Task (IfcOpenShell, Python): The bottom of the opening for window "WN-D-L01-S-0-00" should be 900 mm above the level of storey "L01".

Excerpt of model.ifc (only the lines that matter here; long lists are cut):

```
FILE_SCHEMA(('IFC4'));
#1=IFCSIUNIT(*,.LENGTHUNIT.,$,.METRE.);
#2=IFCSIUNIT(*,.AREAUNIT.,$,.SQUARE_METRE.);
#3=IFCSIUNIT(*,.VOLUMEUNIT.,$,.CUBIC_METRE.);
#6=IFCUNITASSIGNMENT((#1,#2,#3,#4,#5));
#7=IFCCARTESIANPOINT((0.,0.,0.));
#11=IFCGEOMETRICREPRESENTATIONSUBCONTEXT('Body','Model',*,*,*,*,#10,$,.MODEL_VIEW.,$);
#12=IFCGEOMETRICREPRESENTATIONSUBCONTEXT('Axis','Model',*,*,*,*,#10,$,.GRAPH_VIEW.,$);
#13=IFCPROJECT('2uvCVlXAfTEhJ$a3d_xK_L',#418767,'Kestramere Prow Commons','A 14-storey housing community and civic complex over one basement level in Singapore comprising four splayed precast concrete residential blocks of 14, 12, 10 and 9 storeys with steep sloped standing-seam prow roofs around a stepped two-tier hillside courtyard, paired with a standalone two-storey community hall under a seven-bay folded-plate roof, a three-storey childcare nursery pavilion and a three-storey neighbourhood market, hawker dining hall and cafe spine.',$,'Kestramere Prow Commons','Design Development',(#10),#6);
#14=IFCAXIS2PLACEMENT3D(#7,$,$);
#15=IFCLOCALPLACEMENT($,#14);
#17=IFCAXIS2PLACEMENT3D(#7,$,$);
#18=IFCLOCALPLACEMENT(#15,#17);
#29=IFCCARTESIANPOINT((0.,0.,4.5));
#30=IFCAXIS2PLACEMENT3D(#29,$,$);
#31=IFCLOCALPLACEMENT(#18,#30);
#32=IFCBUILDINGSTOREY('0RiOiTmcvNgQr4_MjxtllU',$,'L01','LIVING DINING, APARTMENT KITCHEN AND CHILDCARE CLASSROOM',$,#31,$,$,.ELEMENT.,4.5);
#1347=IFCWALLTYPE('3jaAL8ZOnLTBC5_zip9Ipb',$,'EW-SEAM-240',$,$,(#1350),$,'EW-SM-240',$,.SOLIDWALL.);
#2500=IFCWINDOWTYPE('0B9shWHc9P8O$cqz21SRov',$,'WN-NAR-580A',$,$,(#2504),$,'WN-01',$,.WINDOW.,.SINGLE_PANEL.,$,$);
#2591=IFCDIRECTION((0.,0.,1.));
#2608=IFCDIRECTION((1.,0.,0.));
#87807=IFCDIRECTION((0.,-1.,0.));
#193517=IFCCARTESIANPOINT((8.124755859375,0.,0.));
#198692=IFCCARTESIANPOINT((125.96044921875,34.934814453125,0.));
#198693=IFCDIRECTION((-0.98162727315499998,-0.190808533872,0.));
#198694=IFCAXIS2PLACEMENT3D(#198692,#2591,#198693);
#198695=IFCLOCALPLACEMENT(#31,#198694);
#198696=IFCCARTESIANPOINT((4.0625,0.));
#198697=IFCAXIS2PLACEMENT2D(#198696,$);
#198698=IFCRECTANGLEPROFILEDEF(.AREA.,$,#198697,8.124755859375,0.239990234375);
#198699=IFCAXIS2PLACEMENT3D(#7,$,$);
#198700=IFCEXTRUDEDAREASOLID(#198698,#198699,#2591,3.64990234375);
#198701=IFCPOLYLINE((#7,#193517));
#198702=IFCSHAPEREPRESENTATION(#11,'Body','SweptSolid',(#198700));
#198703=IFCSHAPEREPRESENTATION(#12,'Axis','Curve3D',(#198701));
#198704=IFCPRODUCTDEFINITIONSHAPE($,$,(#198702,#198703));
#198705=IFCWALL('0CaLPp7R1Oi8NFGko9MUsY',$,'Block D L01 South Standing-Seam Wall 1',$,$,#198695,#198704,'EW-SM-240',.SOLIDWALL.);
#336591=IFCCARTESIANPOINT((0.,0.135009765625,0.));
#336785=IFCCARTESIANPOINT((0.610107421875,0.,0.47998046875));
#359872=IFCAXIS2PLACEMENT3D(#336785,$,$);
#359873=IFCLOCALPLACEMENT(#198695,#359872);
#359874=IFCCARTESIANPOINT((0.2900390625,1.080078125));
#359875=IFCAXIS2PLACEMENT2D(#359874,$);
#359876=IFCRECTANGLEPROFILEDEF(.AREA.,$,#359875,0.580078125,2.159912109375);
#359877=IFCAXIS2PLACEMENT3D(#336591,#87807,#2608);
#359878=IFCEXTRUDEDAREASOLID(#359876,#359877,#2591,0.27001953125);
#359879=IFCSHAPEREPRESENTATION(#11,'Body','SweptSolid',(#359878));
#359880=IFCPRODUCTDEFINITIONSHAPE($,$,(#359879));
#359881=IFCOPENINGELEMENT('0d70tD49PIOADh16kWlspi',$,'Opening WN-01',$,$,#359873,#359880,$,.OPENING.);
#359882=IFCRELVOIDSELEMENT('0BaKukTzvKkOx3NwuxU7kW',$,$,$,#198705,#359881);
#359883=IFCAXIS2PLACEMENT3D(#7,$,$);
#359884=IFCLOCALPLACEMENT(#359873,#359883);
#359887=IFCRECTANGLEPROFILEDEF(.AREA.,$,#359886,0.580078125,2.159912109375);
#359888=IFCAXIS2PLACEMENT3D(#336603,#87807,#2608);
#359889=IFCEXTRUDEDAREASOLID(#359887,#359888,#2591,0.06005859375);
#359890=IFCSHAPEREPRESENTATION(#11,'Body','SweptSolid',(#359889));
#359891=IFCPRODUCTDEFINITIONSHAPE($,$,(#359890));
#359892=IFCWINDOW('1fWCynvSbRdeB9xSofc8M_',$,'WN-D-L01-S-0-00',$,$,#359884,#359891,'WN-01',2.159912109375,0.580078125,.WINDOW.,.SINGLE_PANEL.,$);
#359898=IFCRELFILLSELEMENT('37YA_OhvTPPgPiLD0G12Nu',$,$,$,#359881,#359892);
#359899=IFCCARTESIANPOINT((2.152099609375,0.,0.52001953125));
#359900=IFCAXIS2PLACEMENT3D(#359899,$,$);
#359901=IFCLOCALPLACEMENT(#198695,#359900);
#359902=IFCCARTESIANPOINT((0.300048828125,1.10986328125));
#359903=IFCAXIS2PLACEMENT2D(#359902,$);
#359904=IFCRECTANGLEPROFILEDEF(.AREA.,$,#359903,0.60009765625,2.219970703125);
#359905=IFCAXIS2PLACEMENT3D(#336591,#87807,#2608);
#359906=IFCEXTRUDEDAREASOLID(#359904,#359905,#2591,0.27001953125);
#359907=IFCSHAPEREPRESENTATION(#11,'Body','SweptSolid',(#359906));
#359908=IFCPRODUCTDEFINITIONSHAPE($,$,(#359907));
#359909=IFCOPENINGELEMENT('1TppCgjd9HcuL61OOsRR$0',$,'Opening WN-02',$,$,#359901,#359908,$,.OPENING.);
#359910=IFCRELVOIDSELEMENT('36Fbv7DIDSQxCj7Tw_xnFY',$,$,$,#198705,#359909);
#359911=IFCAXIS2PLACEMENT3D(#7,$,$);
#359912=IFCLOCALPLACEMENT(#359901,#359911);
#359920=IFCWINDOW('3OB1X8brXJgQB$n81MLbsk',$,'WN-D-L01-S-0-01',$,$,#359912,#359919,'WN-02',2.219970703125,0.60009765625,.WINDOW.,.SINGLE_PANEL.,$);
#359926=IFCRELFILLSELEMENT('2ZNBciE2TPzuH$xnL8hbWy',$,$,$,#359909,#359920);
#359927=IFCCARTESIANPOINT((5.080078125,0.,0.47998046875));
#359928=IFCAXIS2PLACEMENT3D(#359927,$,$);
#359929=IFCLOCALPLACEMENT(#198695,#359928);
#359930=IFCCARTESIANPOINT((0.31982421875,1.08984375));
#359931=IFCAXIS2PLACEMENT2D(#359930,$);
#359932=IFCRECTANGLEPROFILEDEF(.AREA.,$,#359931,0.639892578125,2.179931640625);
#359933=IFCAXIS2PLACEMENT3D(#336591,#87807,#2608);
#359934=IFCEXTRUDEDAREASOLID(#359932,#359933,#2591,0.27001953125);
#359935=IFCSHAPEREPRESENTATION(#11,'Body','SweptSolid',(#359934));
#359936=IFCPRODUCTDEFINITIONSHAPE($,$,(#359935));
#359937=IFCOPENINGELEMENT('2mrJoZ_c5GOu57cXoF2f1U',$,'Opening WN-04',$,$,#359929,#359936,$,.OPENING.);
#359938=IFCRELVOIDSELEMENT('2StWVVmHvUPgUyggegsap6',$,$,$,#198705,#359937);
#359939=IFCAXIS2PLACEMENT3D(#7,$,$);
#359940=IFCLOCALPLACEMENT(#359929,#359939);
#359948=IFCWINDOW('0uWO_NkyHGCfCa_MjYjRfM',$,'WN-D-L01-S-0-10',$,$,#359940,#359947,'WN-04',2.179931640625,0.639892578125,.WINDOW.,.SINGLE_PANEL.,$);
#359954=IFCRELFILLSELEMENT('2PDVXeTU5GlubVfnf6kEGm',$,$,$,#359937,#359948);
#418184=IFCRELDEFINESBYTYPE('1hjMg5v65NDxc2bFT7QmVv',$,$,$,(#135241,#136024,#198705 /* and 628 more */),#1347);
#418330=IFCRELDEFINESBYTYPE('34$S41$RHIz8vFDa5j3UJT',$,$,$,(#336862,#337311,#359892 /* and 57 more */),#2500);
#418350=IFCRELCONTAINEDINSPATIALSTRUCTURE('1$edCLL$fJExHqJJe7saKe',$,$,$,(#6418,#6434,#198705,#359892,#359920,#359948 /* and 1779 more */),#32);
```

```python
import numpy as np
import ifcopenshell
import ifcopenshell.api.geometry
import ifcopenshell.geom
import ifcopenshell.util.element
import ifcopenshell.util.placement
import ifcopenshell.util.shape
import ifcopenshell.util.unit

model = ifcopenshell.open("model.ifc")
unit_scale = ifcopenshell.util.unit.calculate_unit_scale(model)

window = model.by_id(359892)
opening = window.FillsVoids[0].RelatingOpeningElement
storey = ifcopenshell.util.element.get_container(window, ifc_class="IfcBuildingStorey")
level = ifcopenshell.util.placement.get_local_placement(storey.ObjectPlacement)[2, 3]

# The opening's origin need not be at the sill, so measure its lowest point.
shape = ifcopenshell.geom.create_shape(ifcopenshell.geom.settings(), opening)
bottom = ifcopenshell.util.shape.get_shape_bottom_elevation(shape, shape.geometry) / unit_scale
dz = level + 0.9 - bottom

shift = np.array([0.0, 0.0, dz])
# The window is placed relative to its opening, so it follows when the opening moves.
matrix = ifcopenshell.util.placement.get_local_placement(opening.ObjectPlacement)
matrix[:3, 3] += shift
ifcopenshell.api.geometry.edit_object_placement(
    model, product=opening, matrix=matrix, is_si=False, should_transform_children=True
)

print(f"moved by {dz * unit_scale:+.3f} m")

model.write("model_edited.ifc")
```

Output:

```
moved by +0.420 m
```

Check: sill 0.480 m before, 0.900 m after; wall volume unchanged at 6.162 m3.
